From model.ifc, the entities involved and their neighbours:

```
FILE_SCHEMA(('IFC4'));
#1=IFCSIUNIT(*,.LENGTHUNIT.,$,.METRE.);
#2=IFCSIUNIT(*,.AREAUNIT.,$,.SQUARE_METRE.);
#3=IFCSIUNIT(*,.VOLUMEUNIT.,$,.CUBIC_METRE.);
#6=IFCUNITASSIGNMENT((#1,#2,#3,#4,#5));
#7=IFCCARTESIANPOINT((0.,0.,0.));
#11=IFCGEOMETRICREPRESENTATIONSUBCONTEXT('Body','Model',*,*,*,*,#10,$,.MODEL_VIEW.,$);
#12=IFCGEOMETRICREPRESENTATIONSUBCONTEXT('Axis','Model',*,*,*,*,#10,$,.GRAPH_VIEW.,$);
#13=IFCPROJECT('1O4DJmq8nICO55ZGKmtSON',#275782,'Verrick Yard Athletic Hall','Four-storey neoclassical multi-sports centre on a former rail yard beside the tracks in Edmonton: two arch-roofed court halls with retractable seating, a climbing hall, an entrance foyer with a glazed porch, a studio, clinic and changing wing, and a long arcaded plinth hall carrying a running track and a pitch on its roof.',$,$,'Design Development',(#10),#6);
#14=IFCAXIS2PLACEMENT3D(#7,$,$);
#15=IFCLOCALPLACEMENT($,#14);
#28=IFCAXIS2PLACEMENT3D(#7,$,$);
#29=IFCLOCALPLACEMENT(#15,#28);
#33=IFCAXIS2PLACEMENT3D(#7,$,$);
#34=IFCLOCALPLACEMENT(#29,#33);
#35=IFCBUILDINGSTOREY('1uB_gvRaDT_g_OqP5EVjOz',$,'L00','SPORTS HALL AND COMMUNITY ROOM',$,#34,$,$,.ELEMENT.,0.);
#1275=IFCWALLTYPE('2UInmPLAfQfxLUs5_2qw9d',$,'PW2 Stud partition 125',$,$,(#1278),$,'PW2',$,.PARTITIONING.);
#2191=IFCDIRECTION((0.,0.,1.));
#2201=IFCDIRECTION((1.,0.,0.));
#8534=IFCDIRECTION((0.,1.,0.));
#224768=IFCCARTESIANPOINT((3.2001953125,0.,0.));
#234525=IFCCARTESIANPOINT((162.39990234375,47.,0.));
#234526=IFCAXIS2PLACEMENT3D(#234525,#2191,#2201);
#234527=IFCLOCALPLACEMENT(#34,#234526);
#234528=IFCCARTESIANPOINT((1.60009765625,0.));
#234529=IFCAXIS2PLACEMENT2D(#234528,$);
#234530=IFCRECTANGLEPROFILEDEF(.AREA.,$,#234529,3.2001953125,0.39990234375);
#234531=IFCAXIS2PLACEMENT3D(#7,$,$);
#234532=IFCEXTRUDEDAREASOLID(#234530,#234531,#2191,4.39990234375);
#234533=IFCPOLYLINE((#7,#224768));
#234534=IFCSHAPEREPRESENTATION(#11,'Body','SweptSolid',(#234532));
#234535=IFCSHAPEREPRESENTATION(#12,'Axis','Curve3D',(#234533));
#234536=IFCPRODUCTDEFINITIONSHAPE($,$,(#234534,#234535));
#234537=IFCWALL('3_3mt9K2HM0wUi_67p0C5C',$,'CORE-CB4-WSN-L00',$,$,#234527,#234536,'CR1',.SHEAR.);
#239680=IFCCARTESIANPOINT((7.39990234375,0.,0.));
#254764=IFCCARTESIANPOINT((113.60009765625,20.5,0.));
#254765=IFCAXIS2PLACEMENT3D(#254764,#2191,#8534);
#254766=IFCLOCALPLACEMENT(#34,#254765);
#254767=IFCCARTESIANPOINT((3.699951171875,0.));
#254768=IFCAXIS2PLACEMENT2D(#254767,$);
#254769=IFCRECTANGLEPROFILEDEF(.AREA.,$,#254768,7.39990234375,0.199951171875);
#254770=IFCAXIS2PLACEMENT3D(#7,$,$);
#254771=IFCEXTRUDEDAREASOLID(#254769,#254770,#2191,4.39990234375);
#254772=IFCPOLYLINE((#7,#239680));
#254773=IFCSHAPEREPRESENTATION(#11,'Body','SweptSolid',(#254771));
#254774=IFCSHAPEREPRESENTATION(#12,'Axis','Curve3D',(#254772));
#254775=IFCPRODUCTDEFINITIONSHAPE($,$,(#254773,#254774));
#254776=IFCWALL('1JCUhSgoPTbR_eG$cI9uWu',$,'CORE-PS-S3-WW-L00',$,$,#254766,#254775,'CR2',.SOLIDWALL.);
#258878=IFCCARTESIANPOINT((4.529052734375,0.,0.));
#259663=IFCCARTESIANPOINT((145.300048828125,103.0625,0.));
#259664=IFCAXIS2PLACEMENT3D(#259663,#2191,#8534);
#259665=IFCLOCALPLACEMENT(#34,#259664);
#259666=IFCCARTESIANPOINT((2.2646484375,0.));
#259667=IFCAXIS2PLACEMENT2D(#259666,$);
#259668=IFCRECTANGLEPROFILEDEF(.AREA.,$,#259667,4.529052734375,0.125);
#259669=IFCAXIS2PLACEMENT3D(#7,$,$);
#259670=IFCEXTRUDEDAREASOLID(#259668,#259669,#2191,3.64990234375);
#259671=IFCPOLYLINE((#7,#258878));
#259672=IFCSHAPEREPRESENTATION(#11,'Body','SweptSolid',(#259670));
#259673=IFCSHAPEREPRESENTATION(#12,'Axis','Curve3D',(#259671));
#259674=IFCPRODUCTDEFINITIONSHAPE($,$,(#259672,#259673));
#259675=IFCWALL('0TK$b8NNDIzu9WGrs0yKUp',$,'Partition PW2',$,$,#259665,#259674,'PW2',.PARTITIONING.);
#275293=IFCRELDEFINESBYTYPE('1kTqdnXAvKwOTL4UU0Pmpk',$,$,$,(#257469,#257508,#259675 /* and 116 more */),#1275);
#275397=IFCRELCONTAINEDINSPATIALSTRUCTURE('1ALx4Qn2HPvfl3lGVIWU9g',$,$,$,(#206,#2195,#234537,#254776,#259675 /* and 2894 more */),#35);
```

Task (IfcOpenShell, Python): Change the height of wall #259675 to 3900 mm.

```python
import ifcopenshell
import ifcopenshell.geom
import ifcopenshell.util.representation
import ifcopenshell.util.shape

model = ifcopenshell.open("model.ifc")
settings = ifcopenshell.geom.settings()


def volume(element):
    """Net volume in cubic metres, openings subtracted."""
    shape = ifcopenshell.geom.create_shape(settings, element)
    return ifcopenshell.util.shape.get_volume(shape.geometry)


wall = model.by_guid("0TK$b8NNDIzu9WGrs0yKUp")
before = volume(wall)

body = ifcopenshell.util.representation.get_representation(wall, "Model", "Body")
solid = body.Items[0]
old_height = solid.Depth
solid.Depth = 3.9
after = volume(wall)

print(f"height {old_height:g} -> {solid.Depth:g}, volume {before:.3f} -> {after:.3f} m3")

model.write("model_rev.ifc")
```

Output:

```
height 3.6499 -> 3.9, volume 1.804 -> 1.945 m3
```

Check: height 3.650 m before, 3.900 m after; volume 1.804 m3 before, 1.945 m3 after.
